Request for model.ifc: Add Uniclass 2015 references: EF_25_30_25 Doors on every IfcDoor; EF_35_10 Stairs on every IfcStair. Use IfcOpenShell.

First a look at what the model holds.

```python
import ifcopenshell

model = ifcopenshell.open("model.ifc")
print(model.schema)
print("classifications:", [c.Name for c in model.by_type("IfcClassification")])
for ifc_class in ("IfcDoor", "IfcRoof", "IfcStair", "IfcWall", "IfcWindow"):
    print(ifc_class, len(model.by_type(ifc_class)))
```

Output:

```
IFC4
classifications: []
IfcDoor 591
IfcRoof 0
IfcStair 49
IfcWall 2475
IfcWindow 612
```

```python
import ifcopenshell
import ifcopenshell.api.classification

model = ifcopenshell.open("model.ifc")

system = ifcopenshell.api.classification.add_classification(model, classification="Uniclass 2015")

codes = {
    "IfcDoor": ("EF_25_30_25", "Doors"),
    "IfcStair": ("EF_35_10", "Stairs"),
}
for ifc_class, (code, name) in codes.items():
    products = model.by_type(ifc_class)
    ifcopenshell.api.classification.add_reference(
        model, products=products, classification=system, identification=code, name=name
    )
    print(code, len(products))

model.write("model-out.ifc")
```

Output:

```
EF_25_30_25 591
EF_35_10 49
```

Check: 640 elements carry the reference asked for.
